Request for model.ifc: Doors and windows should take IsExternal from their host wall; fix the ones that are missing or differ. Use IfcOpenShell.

First a look at what the model holds.

```python
import ifcopenshell
import ifcopenshell.util.element

model = ifcopenshell.open("model.ifc")
print(model.schema)
seen = {}
for e in model.by_type("IfcDoor") + model.by_type("IfcWindow"):
    if not e.FillsVoids:
        continue
    host = e.FillsVoids[0].RelatingOpeningElement.VoidsElements[0].RelatingBuildingElement
    own = ifcopenshell.util.element.get_pset(e, f"Pset_{e.is_a()[3:].removesuffix('StandardCase')}Common", "IsExternal")
    wall = ifcopenshell.util.element.get_pset(host, "Pset_WallCommon", "IsExternal")
    seen[e.is_a(), own, wall] = seen.get((e.is_a(), own, wall), 0) + 1
for (cls, own, wall), count in sorted(seen.items(), key=str):
    print(count, cls, "IsExternal:", own, "| host wall:", wall)
```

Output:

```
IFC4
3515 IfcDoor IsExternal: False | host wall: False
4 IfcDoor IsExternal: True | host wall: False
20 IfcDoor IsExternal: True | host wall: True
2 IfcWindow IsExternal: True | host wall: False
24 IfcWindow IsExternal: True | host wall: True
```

```python
import ifcopenshell
import ifcopenshell.api.pset
import ifcopenshell.util.element

model = ifcopenshell.open("model.ifc")

count = 0
for ifc_class, pset_name in (("IfcDoor", "Pset_DoorCommon"), ("IfcWindow", "Pset_WindowCommon")):
    for e in model.by_type(ifc_class):
        if not e.FillsVoids:
            continue
        host = e.FillsVoids[0].RelatingOpeningElement.VoidsElements[0].RelatingBuildingElement
        external = ifcopenshell.util.element.get_pset(host, "Pset_WallCommon", "IsExternal")
        if external is None or ifcopenshell.util.element.get_pset(e, pset_name, "IsExternal") == external:
            continue
        pset = ifcopenshell.api.pset.add_pset(model, product=e, name=pset_name)
        ifcopenshell.api.pset.edit_pset(model, pset=pset, properties={"IsExternal": external})
        count += 1

print(count, "updated")

model.write("model-out.ifc")
```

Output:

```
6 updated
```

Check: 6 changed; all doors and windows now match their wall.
